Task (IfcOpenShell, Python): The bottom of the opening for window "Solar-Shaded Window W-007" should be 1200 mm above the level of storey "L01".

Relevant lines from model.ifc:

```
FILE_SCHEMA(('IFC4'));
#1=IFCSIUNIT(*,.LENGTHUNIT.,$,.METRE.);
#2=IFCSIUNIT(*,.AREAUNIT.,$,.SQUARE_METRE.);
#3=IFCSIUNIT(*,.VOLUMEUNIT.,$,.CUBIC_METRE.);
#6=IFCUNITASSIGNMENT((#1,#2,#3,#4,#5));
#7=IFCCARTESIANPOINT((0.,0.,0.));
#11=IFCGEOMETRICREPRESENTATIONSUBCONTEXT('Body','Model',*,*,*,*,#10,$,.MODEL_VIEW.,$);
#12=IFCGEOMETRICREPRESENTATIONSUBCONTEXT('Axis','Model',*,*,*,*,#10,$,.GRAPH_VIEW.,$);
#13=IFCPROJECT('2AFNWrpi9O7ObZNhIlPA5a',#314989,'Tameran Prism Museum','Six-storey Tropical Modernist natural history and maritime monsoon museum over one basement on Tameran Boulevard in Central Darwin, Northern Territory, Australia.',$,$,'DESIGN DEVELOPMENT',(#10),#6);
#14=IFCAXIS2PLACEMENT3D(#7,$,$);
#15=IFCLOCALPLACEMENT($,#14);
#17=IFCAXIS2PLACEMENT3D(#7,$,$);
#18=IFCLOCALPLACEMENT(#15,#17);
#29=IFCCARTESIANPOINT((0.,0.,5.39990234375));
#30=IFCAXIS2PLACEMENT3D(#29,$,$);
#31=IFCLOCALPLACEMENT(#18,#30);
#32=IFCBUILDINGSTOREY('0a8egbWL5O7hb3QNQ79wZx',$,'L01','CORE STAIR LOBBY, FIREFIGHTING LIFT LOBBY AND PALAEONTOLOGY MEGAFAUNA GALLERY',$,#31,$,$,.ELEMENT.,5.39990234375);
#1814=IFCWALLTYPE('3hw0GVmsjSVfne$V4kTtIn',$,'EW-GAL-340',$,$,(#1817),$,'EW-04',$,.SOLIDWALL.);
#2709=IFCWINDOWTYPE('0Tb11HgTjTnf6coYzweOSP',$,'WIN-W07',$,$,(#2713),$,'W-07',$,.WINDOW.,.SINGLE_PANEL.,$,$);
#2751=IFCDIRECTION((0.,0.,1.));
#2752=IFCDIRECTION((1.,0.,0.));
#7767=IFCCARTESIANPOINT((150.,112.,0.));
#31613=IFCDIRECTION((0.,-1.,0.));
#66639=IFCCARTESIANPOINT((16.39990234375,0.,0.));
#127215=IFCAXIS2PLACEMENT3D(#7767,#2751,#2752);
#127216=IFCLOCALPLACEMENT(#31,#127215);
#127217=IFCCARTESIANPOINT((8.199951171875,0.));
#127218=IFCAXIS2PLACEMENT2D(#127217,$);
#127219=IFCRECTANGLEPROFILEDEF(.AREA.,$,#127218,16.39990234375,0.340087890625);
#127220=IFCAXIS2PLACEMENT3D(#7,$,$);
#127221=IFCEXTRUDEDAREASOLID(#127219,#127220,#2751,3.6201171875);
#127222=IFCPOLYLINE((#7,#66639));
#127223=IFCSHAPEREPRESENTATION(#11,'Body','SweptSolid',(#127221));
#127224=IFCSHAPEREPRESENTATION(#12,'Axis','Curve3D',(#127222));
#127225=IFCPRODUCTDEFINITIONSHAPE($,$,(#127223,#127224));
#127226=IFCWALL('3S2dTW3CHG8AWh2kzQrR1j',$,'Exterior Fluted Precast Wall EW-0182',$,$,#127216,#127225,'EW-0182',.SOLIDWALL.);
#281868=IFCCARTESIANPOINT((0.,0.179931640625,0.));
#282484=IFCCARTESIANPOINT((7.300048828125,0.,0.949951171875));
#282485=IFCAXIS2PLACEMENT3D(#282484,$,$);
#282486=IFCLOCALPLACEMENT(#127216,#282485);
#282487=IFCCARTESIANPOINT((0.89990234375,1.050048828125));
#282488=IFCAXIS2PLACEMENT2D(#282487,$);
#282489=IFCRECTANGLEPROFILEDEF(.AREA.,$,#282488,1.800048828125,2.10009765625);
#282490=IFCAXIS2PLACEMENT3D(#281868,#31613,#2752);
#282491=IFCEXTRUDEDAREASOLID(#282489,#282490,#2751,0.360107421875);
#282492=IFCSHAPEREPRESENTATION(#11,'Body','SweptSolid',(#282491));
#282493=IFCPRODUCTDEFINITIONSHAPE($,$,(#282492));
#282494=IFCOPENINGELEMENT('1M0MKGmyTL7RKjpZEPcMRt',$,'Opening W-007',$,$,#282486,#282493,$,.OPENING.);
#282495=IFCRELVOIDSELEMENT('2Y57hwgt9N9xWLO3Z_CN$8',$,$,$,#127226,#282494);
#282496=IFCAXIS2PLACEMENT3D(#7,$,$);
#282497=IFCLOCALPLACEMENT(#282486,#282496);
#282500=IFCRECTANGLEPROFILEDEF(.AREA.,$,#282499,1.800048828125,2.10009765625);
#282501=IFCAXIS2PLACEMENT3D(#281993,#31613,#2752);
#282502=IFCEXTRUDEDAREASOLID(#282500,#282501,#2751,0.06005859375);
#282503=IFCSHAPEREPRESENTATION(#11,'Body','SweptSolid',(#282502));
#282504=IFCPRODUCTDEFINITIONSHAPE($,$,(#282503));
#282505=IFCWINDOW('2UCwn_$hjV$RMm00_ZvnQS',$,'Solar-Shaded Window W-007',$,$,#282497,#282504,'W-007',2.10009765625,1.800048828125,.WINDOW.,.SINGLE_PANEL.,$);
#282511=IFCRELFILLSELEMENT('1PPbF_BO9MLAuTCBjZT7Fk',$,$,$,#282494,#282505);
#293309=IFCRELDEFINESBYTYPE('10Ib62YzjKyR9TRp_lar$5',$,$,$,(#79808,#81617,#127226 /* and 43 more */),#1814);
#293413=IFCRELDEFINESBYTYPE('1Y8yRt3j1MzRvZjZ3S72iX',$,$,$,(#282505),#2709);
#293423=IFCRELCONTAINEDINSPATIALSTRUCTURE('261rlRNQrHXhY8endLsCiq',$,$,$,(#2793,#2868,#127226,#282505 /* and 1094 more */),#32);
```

```python
import numpy as np
import ifcopenshell
import ifcopenshell.api.geometry
import ifcopenshell.geom
import ifcopenshell.util.element
import ifcopenshell.util.placement
import ifcopenshell.util.shape
import ifcopenshell.util.unit

model = ifcopenshell.open("model.ifc")
unit_scale = ifcopenshell.util.unit.calculate_unit_scale(model)

window = model.by_guid("2UCwn_$hjV$RMm00_ZvnQS")
opening = window.FillsVoids[0].RelatingOpeningElement
storey = ifcopenshell.util.element.get_container(window, ifc_class="IfcBuildingStorey")
level = ifcopenshell.util.placement.get_local_placement(storey.ObjectPlacement)[2, 3]

# The opening's origin need not be at the sill, so measure its lowest point.
shape = ifcopenshell.geom.create_shape(ifcopenshell.geom.settings(), opening)
bottom = ifcopenshell.util.shape.get_shape_bottom_elevation(shape, shape.geometry) / unit_scale
dz = level + 1.2 - bottom

shift = np.array([0.0, 0.0, dz])
# The window is placed relative to its opening, so it follows when the opening moves.
matrix = ifcopenshell.util.placement.get_local_placement(opening.ObjectPlacement)
matrix[:3, 3] += shift
ifcopenshell.api.geometry.edit_object_placement(
    model, product=opening, matrix=matrix, is_si=False, should_transform_children=True
)

print(f"moved by {dz * unit_scale:+.3f} m")

model.write("model-out.ifc")
```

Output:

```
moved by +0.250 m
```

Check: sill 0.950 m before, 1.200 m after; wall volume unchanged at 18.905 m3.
